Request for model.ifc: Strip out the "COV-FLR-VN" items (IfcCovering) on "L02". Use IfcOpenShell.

First a look at what the model holds.

```python
import ifcopenshell
import ifcopenshell.util.element

model = ifcopenshell.open("model.ifc")
print(model.schema)
storey = next(s for s in model.by_type("IfcBuildingStorey") if s.Name == "L02")
coverings = [e for e in ifcopenshell.util.element.get_decomposition(storey) if e.is_a("IfcCovering")]
seen = {}
for e in coverings:
    element_type = ifcopenshell.util.element.get_type(e)
    name = element_type.Name if element_type not in (None, e) else None
    seen[name] = seen.get(name, 0) + 1
for name, count in sorted(seen.items(), key=str):
    print(count, "x", name)
```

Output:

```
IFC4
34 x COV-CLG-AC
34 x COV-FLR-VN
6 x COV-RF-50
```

```python
import ifcopenshell
import ifcopenshell.api.root
import ifcopenshell.util.element

model = ifcopenshell.open("model.ifc")

storey = next(s for s in model.by_type("IfcBuildingStorey") if s.Name == "L02")
coverings = [e for e in ifcopenshell.util.element.get_decomposition(storey) if e.is_a("IfcCovering")]
targets = [e for e in coverings if (t := ifcopenshell.util.element.get_type(e)) not in (None, e) and t.Name == "COV-FLR-VN"]

for e in targets:
    ifcopenshell.api.root.remove_product(model, product=e)
print(len(targets), "removed")

model.write("model_edited.ifc")
```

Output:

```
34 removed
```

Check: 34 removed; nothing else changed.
